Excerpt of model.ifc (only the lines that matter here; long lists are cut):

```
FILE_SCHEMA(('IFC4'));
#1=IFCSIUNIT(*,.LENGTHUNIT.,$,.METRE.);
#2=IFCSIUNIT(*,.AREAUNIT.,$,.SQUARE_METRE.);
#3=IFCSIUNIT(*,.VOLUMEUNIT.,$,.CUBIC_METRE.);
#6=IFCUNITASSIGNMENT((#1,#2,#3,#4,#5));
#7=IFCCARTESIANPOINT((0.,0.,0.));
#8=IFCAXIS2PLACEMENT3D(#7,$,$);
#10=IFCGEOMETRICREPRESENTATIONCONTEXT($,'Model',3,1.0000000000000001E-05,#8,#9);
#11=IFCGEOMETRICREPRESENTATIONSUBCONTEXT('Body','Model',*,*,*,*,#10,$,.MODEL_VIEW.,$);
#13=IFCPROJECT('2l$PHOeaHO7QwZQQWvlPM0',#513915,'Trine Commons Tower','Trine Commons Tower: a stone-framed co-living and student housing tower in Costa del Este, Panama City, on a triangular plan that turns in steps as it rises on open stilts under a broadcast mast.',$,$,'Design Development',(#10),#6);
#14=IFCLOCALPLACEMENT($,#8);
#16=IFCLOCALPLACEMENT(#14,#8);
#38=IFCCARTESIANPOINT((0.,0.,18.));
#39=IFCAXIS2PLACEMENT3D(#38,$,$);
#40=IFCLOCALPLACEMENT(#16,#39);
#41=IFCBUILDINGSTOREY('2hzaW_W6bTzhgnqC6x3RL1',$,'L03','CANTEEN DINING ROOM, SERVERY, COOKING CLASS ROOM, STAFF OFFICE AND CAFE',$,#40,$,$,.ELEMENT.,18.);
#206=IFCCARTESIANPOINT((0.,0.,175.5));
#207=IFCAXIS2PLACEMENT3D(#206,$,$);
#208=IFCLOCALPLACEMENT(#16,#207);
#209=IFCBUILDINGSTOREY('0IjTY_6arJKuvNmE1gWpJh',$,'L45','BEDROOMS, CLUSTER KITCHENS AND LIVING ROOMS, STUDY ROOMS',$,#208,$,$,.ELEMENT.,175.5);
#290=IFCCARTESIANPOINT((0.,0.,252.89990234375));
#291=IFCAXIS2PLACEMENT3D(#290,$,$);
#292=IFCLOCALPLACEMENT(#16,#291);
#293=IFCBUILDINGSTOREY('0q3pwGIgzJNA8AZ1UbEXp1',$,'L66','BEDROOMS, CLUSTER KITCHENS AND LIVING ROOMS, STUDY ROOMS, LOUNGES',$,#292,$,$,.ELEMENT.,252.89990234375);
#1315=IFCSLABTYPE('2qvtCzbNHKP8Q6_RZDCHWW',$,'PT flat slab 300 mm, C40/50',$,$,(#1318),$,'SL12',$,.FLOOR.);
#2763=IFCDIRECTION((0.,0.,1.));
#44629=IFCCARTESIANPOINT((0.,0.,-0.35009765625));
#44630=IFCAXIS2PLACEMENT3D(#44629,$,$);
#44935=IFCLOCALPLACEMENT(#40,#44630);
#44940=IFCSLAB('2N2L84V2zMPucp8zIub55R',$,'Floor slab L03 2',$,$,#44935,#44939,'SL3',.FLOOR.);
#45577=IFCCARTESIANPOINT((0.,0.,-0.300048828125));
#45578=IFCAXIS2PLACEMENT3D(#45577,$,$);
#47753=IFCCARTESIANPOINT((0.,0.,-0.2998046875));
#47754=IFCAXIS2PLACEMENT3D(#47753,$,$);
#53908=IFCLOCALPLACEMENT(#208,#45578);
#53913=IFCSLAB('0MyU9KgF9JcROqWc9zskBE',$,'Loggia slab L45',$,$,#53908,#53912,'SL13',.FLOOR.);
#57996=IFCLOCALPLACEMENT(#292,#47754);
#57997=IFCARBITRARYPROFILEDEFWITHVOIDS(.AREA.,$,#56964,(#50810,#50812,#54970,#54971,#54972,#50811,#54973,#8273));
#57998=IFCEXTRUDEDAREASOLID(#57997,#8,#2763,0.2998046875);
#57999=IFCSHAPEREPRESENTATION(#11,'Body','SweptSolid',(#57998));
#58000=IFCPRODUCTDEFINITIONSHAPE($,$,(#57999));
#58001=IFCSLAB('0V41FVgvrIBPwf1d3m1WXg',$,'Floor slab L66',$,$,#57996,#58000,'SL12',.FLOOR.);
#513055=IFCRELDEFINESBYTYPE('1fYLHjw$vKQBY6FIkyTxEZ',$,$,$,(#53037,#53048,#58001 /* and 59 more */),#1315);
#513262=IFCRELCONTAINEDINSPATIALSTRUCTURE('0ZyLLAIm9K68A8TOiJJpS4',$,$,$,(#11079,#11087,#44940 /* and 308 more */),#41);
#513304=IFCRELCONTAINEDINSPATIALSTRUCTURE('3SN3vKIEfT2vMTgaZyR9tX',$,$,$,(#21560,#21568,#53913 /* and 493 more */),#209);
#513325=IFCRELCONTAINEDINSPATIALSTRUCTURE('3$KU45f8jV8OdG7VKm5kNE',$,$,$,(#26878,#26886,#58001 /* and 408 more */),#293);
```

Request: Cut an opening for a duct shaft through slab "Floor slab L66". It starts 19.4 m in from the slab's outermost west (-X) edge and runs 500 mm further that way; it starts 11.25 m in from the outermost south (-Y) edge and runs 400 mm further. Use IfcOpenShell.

```python
import numpy as np
import ifcopenshell
import ifcopenshell.api.feature
import ifcopenshell.api.geometry
import ifcopenshell.api.root
import ifcopenshell.geom
import ifcopenshell.util.placement
import ifcopenshell.util.representation
import ifcopenshell.util.shape
import ifcopenshell.util.unit

model = ifcopenshell.open("model.ifc")
unit_scale = ifcopenshell.util.unit.calculate_unit_scale(model)
settings = ifcopenshell.geom.settings()


def volume(element):
    """Net volume in cubic metres, openings subtracted."""
    shape = ifcopenshell.geom.create_shape(settings, element)
    return ifcopenshell.util.shape.get_volume(shape.geometry)


slab = model.by_guid("0V41FVgvrIBPwf1d3m1WXg")
before = volume(slab)

# Extent in the slab's own axes, in metres. The edges named are its -X and -Y sides.
slab_shape = ifcopenshell.geom.create_shape(settings, slab)
vertices = ifcopenshell.util.shape.get_vertices(slab_shape.geometry)
x_min, y_min, bottom = vertices.min(axis=0)
top = vertices[:, 2].max()

opening = ifcopenshell.api.root.create_entity(model, ifc_class="IfcOpeningElement", name="Duct shaft opening", predefined_type="OPENING")
context = ifcopenshell.util.representation.get_context(model, "Model", "Body", "MODEL_VIEW")
width, depth = 0.5, 0.4
outline = [(0.0, 0.0), (width, 0.0), (width, depth), (0.0, depth), (0.0, 0.0)]
# Overshoot both faces by 50 mm so the cut is clean.
shape = ifcopenshell.api.geometry.add_slab_representation(
    model, context=context, depth=top - bottom + 0.1, polyline=outline
)
ifcopenshell.api.geometry.assign_representation(model, product=opening, representation=shape)

matrix = ifcopenshell.util.placement.get_local_placement(slab.ObjectPlacement)
matrix[:, 3] = matrix @ np.append(np.array([x_min + 19.4, y_min + 11.25, bottom - 0.05]) / unit_scale, 1.0)
ifcopenshell.api.geometry.edit_object_placement(model, product=opening, matrix=matrix, is_si=False)
ifcopenshell.api.feature.add_feature(model, feature=opening, element=slab)

after = volume(slab)

print(f"slab volume {before:.3f} -> {after:.3f} m3")

model.write("model_v2.ifc")
```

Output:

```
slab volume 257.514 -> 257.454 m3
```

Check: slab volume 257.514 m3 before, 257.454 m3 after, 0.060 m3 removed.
